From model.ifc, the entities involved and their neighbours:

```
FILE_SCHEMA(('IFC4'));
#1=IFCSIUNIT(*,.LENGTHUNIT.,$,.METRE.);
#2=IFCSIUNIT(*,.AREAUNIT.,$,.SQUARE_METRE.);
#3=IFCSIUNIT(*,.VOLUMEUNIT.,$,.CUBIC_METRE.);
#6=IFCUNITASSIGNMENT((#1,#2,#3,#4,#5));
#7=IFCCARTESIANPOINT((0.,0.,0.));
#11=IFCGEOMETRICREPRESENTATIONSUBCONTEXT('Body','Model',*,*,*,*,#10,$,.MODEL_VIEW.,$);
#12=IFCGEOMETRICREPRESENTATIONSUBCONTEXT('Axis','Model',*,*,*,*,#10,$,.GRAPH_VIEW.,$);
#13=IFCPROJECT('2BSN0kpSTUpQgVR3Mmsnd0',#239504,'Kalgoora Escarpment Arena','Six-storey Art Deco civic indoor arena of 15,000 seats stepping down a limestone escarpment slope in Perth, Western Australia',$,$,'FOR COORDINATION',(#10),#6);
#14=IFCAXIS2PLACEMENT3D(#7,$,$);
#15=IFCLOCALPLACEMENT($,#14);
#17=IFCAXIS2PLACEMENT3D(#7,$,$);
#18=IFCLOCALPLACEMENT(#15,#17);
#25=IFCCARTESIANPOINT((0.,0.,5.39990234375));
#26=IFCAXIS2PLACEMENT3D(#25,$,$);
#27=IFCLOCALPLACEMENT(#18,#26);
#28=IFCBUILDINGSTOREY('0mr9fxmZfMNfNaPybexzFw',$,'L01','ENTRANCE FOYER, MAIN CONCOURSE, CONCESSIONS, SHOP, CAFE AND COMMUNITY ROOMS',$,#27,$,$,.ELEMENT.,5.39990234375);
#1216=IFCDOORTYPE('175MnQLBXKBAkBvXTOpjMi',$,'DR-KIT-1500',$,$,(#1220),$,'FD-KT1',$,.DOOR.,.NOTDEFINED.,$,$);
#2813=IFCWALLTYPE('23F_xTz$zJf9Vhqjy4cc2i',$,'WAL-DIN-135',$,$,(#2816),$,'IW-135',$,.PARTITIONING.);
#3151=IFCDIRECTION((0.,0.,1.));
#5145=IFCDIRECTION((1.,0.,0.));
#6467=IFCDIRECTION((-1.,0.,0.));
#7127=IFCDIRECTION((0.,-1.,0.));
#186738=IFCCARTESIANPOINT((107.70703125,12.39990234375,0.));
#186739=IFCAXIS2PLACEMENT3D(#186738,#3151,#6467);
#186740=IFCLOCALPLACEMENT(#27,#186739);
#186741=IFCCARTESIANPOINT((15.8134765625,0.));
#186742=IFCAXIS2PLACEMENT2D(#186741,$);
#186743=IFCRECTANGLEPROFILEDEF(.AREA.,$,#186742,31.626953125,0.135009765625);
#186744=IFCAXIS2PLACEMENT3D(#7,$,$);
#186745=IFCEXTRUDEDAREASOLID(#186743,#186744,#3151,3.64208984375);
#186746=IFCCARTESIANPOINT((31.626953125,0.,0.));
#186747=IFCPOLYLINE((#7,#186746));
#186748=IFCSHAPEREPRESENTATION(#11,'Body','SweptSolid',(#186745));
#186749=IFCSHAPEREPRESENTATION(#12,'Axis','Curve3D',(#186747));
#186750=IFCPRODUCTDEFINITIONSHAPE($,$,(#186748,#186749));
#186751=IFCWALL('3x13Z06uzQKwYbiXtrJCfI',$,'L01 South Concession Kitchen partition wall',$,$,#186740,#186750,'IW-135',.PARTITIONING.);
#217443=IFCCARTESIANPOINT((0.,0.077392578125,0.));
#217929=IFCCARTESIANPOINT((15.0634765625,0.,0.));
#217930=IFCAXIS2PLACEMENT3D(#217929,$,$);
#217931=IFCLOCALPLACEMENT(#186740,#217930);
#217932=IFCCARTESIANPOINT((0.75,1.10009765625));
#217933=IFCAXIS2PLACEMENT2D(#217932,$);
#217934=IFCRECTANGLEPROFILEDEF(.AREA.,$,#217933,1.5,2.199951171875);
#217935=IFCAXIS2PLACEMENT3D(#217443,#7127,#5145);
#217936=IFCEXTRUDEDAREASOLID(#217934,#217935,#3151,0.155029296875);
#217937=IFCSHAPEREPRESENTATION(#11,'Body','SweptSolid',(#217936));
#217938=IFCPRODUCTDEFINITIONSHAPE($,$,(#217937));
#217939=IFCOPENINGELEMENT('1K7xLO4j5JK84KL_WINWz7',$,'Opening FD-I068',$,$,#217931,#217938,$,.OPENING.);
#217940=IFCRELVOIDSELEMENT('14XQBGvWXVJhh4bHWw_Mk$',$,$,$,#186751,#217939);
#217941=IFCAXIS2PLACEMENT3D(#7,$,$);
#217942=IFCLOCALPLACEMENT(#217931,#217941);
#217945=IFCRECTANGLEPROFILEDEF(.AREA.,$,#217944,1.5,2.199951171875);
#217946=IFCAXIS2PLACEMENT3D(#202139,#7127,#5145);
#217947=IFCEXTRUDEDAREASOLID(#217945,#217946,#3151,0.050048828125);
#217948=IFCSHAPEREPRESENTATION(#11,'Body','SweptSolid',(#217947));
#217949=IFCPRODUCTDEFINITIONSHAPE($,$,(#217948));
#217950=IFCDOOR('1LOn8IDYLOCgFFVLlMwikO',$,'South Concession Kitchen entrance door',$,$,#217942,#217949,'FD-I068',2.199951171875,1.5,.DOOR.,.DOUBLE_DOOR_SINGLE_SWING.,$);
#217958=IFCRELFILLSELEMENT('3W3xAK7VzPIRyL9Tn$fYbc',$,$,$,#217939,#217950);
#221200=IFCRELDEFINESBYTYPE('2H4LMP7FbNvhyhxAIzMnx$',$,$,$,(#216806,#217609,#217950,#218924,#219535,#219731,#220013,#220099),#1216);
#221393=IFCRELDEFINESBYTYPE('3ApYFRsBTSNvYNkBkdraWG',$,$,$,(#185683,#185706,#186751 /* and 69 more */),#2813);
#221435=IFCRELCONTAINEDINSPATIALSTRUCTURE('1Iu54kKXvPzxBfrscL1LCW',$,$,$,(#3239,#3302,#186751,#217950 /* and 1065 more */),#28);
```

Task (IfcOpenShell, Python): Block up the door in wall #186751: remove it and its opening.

```python
import ifcopenshell
import ifcopenshell.api.feature
import ifcopenshell.api.root
import ifcopenshell.geom
import ifcopenshell.util.shape

model = ifcopenshell.open("model.ifc")
settings = ifcopenshell.geom.settings()


def volume(element):
    """Net volume in cubic metres, openings subtracted."""
    shape = ifcopenshell.geom.create_shape(settings, element)
    return ifcopenshell.util.shape.get_volume(shape.geometry)


door = model.by_guid("1LOn8IDYLOCgFFVLlMwikO")
opening = door.FillsVoids[0].RelatingOpeningElement
wall = opening.VoidsElements[0].RelatingBuildingElement
before = volume(wall)

ifcopenshell.api.root.remove_product(model, product=door)
ifcopenshell.api.feature.remove_feature(model, feature=opening)

after = volume(wall)

print(f"wall volume {before:.3f} -> {after:.3f} m3")

model.write("model_edited.ifc")
```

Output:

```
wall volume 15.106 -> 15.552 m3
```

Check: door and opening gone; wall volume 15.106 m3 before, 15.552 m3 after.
